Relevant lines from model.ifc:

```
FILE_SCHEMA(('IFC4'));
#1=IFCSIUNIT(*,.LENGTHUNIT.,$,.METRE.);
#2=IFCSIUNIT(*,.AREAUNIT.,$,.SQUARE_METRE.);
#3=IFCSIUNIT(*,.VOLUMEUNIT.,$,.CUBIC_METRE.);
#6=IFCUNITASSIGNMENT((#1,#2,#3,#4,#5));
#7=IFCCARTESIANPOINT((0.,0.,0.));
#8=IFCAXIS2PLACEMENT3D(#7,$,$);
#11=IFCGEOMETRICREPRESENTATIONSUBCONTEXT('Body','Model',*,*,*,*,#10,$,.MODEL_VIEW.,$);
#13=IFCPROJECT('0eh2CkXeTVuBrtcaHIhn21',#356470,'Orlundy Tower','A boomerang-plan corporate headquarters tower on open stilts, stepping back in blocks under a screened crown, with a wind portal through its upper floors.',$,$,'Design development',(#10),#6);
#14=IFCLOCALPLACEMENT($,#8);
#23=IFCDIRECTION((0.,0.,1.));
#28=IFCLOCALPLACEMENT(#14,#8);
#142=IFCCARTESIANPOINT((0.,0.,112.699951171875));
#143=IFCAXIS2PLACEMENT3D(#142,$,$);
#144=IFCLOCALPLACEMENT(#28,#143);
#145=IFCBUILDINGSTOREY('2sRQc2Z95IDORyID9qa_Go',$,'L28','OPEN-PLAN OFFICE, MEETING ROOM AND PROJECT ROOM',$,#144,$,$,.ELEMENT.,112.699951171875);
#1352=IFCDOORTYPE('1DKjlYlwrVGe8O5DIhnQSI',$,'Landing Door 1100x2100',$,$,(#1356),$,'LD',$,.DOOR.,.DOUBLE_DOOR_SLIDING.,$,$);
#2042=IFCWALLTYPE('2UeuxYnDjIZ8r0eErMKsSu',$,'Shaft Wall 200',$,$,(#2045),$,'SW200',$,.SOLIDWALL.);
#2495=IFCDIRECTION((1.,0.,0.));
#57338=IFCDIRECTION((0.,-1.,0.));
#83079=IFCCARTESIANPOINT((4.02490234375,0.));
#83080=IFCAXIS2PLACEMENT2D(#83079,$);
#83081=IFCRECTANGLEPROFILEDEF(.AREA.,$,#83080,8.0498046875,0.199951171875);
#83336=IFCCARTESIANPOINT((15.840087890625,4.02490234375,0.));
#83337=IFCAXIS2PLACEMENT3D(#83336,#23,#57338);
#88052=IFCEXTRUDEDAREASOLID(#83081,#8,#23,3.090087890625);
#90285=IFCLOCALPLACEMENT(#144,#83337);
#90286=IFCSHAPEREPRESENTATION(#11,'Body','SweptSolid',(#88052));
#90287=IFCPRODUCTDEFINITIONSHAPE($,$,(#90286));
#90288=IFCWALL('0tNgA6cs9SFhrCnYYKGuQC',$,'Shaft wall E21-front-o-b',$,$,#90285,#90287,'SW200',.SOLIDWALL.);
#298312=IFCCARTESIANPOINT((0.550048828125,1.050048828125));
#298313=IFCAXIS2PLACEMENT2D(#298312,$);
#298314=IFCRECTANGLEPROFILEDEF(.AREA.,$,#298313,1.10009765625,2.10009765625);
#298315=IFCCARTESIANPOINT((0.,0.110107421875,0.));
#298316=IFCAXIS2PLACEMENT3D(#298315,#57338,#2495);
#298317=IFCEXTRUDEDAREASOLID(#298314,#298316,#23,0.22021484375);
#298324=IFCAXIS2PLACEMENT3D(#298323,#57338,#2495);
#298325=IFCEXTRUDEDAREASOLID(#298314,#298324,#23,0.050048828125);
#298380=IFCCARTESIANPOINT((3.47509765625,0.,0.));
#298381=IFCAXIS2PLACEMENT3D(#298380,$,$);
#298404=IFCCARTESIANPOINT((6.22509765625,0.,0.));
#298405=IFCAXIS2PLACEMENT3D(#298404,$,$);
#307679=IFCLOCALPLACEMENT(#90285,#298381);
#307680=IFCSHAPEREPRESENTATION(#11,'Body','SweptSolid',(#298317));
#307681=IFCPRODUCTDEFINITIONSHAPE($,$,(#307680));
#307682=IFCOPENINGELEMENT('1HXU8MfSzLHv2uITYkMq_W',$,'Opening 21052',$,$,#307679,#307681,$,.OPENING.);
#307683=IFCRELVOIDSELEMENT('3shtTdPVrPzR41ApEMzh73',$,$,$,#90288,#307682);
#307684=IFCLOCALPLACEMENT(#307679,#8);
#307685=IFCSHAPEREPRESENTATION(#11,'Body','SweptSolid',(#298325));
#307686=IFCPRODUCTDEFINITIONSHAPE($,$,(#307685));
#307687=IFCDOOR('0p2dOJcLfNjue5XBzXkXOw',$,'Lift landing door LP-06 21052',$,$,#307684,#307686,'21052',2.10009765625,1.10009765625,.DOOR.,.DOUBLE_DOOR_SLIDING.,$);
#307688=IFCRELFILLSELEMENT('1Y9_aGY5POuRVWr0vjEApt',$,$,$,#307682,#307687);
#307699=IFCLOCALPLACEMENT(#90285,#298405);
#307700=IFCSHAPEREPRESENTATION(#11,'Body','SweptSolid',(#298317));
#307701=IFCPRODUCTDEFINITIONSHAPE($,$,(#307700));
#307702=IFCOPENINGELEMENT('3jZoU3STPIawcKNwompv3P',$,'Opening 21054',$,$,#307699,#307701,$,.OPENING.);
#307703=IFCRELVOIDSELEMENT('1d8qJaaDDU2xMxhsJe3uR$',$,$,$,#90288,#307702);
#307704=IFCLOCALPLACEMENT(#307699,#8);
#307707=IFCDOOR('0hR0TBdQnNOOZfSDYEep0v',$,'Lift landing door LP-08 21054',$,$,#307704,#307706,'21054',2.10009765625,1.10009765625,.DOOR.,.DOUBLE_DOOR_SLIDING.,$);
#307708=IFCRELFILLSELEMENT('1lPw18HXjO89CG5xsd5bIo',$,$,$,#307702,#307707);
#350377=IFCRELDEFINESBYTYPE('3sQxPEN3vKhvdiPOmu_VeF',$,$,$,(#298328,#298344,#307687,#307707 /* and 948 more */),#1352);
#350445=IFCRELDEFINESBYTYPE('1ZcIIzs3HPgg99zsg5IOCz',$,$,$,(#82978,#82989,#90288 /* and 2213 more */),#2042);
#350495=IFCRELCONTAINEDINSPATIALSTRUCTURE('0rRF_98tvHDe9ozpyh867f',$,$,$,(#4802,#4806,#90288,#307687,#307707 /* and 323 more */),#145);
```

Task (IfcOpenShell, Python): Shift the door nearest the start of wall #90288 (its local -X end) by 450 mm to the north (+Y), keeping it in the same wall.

```python
import ifcopenshell
import ifcopenshell.api.geometry
import ifcopenshell.util.placement

model = ifcopenshell.open("model.ifc")

door = model.by_id(307687)
opening = door.FillsVoids[0].RelatingOpeningElement
wall = opening.VoidsElements[0].RelatingBuildingElement

wall_matrix = ifcopenshell.util.placement.get_local_placement(wall.ObjectPlacement)
shift = wall_matrix[:3, 0] * -0.45
before = ifcopenshell.util.placement.get_local_placement(door.ObjectPlacement)[:3, 3].copy()

# The door is placed relative to its opening, so it follows when the opening moves.
matrix = ifcopenshell.util.placement.get_local_placement(opening.ObjectPlacement)
matrix[:3, 3] += shift
ifcopenshell.api.geometry.edit_object_placement(
    model, product=opening, matrix=matrix, is_si=False, should_transform_children=True
)

after = ifcopenshell.util.placement.get_local_placement(door.ObjectPlacement)[:3, 3]
print("door moved by", (after - before).round(3) + 0.0)

model.write("model_v2.ifc")
```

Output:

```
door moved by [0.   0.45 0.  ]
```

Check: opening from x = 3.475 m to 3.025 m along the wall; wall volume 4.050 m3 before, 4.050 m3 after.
